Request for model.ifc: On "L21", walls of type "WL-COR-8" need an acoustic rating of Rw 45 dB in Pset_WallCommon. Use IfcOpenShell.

First a look at what the model holds.

```python
import ifcopenshell
import ifcopenshell.util.element

model = ifcopenshell.open("model.ifc")
print(model.schema)
storey = next(s for s in model.by_type("IfcBuildingStorey") if s.Name == "L21")
walls = [e for e in ifcopenshell.util.element.get_decomposition(storey) if e.is_a("IfcWall")]
seen = {}
for e in walls:
    element_type = ifcopenshell.util.element.get_type(e)
    key = (element_type.Name if element_type != e and element_type else None, ifcopenshell.util.element.get_pset(e, "Pset_WallCommon", "AcousticRating"))
    seen[key] = seen.get(key, 0) + 1
for (name, value), count in sorted(seen.items(), key=str):
    print(count, "x", name, "|", value)
```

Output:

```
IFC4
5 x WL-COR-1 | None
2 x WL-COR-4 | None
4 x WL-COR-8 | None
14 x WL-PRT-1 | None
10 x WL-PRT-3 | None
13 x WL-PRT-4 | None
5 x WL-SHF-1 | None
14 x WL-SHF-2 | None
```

```python
import ifcopenshell
import ifcopenshell.api.pset
import ifcopenshell.util.element

model = ifcopenshell.open("model.ifc")

storey = next(s for s in model.by_type("IfcBuildingStorey") if s.Name == "L21")
walls = [e for e in ifcopenshell.util.element.get_decomposition(storey) if e.is_a("IfcWall")]

count = 0
for e in walls:
    element_type = ifcopenshell.util.element.get_type(e)
    if element_type in (None, e) or element_type.Name != "WL-COR-8":
        continue
    # add_pset returns the element's existing set when there is one.
    pset = ifcopenshell.api.pset.add_pset(model, product=e, name="Pset_WallCommon")
    ifcopenshell.api.pset.edit_pset(model, pset=pset, properties={"AcousticRating": "Rw 45 dB"})
    count += 1

print(count, "walls updated")

model.write("model_updated.ifc")
```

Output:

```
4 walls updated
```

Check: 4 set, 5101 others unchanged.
